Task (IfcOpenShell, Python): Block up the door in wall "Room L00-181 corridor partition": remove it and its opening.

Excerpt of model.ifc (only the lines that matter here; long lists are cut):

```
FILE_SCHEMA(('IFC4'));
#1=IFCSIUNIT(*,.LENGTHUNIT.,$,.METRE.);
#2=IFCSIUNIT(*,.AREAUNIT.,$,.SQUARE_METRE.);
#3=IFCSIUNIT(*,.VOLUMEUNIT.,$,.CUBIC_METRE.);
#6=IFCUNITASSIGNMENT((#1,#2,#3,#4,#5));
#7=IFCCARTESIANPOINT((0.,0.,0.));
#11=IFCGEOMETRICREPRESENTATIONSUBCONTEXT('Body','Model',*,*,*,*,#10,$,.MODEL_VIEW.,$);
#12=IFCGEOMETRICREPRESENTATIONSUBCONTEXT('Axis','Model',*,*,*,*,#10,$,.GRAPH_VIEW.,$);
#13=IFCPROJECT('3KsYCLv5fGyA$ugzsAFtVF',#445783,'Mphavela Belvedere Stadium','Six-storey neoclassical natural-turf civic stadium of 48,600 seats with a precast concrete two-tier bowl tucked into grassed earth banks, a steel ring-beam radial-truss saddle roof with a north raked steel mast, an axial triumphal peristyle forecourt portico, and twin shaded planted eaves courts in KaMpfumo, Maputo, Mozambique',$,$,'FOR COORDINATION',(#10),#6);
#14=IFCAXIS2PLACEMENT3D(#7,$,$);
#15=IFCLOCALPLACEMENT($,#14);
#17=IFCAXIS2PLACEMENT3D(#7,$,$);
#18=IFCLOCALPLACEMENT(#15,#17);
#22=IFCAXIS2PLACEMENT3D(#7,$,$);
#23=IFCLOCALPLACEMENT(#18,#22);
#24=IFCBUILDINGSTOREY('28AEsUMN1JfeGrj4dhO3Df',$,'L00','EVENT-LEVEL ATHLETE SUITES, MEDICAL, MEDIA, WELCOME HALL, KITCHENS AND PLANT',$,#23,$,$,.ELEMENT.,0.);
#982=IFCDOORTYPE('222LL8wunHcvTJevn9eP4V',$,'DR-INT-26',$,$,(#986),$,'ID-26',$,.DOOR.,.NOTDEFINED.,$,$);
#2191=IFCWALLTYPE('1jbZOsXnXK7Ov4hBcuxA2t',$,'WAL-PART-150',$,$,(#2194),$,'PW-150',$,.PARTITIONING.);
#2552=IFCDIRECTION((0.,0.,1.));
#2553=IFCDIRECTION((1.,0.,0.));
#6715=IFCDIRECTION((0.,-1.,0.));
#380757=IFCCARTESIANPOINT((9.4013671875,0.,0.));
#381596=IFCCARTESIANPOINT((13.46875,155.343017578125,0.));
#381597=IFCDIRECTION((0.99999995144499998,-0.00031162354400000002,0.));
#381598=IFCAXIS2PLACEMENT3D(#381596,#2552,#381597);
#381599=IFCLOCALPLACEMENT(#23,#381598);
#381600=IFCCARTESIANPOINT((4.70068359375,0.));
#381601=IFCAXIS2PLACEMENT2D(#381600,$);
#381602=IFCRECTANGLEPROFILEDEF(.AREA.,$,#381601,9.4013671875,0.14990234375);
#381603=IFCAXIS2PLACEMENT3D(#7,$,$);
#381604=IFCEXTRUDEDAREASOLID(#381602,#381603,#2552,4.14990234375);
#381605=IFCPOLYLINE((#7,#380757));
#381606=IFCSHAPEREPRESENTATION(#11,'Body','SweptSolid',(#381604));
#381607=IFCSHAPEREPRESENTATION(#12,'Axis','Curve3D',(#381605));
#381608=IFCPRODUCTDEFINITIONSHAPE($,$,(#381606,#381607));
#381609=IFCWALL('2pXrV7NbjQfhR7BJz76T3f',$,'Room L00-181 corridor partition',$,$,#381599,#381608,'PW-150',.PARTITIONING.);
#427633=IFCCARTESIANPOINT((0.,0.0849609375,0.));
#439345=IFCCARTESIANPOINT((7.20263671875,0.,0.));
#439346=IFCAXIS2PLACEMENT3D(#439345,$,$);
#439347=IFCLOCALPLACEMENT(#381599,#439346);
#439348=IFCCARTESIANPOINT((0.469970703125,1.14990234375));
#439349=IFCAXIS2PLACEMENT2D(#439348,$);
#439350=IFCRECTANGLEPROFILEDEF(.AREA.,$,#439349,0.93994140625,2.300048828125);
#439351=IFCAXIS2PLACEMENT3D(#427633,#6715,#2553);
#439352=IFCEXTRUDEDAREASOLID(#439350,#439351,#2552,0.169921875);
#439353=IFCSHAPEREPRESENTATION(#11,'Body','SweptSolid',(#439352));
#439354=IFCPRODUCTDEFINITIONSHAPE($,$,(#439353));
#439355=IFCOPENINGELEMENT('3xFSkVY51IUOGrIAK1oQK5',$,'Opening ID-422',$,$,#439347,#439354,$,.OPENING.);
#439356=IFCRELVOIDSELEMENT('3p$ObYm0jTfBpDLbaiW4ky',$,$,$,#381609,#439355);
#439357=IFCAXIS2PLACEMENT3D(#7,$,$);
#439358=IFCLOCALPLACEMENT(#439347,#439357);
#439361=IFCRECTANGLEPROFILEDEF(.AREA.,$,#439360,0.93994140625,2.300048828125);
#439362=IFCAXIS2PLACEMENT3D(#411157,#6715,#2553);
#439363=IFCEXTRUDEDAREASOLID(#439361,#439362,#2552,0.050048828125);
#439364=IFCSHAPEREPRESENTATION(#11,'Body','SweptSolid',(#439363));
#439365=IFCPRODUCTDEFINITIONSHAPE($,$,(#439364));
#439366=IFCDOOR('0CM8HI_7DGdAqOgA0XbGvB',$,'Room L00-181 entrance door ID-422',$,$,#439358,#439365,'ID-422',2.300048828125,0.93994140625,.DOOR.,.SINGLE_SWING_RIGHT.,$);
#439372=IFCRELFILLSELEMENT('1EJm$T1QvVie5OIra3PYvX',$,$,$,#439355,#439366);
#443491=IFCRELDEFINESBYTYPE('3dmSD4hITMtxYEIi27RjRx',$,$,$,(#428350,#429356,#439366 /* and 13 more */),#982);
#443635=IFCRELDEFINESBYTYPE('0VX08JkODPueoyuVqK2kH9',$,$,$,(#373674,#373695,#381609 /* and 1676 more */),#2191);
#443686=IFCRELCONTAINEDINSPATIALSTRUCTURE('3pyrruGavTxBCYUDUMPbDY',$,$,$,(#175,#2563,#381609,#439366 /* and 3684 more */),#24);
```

```python
import ifcopenshell
import ifcopenshell.api.feature
import ifcopenshell.api.root
import ifcopenshell.geom
import ifcopenshell.util.shape

model = ifcopenshell.open("model.ifc")
settings = ifcopenshell.geom.settings()


def volume(element):
    """Net volume in cubic metres, openings subtracted."""
    shape = ifcopenshell.geom.create_shape(settings, element)
    return ifcopenshell.util.shape.get_volume(shape.geometry)


door = model.by_guid("0CM8HI_7DGdAqOgA0XbGvB")
opening = door.FillsVoids[0].RelatingOpeningElement
wall = opening.VoidsElements[0].RelatingBuildingElement
before = volume(wall)

ifcopenshell.api.root.remove_product(model, product=door)
ifcopenshell.api.feature.remove_feature(model, feature=opening)

after = volume(wall)

print(f"wall volume {before:.3f} -> {after:.3f} m3")

model.write("model_rev.ifc")
```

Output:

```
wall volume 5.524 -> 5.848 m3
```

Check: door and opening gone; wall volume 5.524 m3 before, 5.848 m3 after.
